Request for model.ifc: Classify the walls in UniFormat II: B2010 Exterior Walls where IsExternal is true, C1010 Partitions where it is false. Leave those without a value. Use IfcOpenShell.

First a look at what the model holds.

```python
import ifcopenshell
import ifcopenshell.util.element

model = ifcopenshell.open("model.ifc")
print(model.schema)
print("classifications:", [c.Name for c in model.by_type("IfcClassification")])
values = [ifcopenshell.util.element.get_pset(e, "Pset_WallCommon", "IsExternal") for e in model.by_type("IfcWall")]
for value in (True, False, None):
    print("IsExternal", value, values.count(value))
```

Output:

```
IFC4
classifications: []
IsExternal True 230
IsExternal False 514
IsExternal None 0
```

```python
import ifcopenshell
import ifcopenshell.api.classification
import ifcopenshell.util.element

model = ifcopenshell.open("model.ifc")

system = ifcopenshell.api.classification.add_classification(model, classification="UniFormat II")

walls = model.by_type("IfcWall")
external = {e: ifcopenshell.util.element.get_pset(e, "Pset_WallCommon", "IsExternal") for e in walls}
for flag, code, name in ((True, "B2010", "Exterior Walls"), (False, "C1010", "Partitions")):
    products = [e for e in walls if external[e] is flag]
    ifcopenshell.api.classification.add_reference(
        model, products=products, classification=system, identification=code, name=name
    )
    print(code, len(products))

model.write("model_updated.ifc")
```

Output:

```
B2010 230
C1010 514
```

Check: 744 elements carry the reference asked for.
